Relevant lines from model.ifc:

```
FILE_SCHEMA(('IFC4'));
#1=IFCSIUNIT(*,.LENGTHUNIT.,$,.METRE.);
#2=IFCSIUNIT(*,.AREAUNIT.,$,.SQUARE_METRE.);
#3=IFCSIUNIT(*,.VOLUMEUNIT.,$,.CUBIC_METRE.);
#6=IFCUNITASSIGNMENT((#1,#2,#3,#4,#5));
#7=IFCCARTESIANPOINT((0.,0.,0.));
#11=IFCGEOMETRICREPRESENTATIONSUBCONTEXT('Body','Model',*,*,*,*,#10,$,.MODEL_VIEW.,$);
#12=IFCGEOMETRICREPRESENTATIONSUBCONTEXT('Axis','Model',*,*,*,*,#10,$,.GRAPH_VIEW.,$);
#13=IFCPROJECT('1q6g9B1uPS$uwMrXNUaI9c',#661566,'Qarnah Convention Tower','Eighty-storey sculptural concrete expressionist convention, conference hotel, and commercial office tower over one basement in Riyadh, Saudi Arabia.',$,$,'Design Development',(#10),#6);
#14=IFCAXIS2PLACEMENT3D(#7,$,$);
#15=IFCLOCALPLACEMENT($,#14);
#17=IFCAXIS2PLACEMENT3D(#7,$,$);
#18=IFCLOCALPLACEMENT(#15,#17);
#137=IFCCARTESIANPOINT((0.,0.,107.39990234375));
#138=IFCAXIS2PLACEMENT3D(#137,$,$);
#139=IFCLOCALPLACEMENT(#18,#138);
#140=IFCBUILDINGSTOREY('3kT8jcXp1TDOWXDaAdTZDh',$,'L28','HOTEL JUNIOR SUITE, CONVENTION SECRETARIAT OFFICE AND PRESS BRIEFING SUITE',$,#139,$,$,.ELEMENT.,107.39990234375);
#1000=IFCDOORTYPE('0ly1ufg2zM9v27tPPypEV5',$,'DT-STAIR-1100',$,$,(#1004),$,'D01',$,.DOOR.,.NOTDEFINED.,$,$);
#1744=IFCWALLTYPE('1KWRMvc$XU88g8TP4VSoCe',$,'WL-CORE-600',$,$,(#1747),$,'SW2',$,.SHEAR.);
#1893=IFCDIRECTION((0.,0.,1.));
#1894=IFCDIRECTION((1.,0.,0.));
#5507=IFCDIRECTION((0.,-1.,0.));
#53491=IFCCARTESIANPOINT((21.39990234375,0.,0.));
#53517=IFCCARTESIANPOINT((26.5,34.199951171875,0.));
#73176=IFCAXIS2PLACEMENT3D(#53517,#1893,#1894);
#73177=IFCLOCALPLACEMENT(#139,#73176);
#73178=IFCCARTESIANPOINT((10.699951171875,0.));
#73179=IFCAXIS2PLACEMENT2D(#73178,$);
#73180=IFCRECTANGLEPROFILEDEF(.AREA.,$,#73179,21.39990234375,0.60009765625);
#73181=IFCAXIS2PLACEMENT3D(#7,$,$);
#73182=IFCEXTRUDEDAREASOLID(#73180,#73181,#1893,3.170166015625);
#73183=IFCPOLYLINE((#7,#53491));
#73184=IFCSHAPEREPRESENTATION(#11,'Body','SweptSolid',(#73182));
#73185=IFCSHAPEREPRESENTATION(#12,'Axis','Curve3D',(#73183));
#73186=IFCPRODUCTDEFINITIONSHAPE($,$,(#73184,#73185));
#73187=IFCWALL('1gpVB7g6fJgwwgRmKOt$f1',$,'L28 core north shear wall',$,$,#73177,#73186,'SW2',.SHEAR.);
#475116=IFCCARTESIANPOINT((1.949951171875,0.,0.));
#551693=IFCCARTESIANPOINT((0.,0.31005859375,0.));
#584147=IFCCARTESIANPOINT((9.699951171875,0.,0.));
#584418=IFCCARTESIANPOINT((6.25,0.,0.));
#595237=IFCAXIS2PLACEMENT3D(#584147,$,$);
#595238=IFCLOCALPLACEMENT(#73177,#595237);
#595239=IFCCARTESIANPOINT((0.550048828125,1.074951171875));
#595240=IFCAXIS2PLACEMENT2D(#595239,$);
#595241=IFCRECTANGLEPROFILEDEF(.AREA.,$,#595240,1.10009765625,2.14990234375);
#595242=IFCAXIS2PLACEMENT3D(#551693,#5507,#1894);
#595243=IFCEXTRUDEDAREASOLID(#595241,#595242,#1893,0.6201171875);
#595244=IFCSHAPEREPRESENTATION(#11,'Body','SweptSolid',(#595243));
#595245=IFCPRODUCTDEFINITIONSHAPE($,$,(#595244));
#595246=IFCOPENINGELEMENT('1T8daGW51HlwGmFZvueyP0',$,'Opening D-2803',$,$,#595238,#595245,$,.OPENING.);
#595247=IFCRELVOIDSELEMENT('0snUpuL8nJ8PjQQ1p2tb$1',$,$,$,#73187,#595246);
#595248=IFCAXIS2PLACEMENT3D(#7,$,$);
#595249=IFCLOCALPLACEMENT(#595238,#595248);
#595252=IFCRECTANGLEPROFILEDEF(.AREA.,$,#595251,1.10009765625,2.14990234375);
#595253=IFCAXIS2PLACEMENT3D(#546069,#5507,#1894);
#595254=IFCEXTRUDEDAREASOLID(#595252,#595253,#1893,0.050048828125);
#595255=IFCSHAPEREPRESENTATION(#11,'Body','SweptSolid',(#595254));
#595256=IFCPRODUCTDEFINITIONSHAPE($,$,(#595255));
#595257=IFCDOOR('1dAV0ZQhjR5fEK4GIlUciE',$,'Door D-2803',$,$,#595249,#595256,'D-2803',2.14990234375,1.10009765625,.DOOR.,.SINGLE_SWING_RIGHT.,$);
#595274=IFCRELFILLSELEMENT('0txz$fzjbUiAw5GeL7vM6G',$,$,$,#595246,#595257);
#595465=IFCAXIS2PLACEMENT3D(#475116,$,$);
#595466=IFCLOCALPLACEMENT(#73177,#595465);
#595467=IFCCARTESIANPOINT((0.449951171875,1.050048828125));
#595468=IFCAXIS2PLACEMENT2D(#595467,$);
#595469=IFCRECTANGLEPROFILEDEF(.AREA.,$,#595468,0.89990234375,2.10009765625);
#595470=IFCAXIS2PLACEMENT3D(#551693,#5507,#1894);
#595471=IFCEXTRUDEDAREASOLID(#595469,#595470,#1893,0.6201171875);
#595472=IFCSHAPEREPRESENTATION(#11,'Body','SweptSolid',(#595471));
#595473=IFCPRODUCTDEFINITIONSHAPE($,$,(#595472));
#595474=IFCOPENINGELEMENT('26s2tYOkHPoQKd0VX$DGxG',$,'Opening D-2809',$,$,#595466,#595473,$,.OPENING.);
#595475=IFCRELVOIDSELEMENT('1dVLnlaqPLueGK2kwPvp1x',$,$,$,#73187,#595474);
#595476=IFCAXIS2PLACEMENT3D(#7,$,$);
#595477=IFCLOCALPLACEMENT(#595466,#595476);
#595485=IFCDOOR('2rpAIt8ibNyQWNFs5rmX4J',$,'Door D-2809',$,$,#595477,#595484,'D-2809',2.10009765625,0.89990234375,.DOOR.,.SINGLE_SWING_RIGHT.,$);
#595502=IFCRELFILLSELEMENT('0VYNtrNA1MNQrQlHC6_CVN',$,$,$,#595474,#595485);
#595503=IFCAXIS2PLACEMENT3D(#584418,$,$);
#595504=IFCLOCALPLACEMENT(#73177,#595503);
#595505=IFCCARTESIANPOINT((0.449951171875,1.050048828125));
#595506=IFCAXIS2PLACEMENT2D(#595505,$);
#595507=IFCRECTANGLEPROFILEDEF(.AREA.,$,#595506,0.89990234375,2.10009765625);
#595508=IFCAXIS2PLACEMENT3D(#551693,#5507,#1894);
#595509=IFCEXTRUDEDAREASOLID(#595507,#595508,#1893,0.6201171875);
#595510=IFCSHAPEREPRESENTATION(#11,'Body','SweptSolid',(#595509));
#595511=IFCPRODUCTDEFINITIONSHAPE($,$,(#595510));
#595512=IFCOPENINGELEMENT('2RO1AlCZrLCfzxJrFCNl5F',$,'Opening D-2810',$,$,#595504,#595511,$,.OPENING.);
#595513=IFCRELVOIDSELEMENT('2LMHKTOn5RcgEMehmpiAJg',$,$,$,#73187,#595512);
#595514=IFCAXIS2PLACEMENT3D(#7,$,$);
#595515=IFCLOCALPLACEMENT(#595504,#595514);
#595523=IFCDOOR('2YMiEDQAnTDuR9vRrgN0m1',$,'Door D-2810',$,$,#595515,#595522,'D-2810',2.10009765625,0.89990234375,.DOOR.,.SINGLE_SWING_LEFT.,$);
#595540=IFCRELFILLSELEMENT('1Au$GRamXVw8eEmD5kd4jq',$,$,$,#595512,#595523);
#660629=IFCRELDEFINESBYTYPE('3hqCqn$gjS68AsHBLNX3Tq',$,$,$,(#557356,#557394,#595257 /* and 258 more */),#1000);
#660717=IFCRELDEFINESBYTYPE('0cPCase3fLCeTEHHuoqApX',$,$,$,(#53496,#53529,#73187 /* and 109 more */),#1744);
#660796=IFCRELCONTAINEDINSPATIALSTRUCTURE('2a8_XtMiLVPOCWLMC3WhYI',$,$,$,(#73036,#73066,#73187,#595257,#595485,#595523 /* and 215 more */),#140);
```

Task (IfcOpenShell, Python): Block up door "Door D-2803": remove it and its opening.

```python
import ifcopenshell
import ifcopenshell.api.feature
import ifcopenshell.api.root
import ifcopenshell.geom
import ifcopenshell.util.shape

model = ifcopenshell.open("model.ifc")
settings = ifcopenshell.geom.settings()


def volume(element):
    """Net volume in cubic metres, openings subtracted."""
    shape = ifcopenshell.geom.create_shape(settings, element)
    return ifcopenshell.util.shape.get_volume(shape.geometry)


door = model.by_guid("1dAV0ZQhjR5fEK4GIlUciE")
opening = door.FillsVoids[0].RelatingOpeningElement
wall = opening.VoidsElements[0].RelatingBuildingElement
before = volume(wall)

ifcopenshell.api.root.remove_product(model, product=door)
ifcopenshell.api.feature.remove_feature(model, feature=opening)

after = volume(wall)

print(f"wall volume {before:.3f} -> {after:.3f} m3")

model.write("model_rev.ifc")
```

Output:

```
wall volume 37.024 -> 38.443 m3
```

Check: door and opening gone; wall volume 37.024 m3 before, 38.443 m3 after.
